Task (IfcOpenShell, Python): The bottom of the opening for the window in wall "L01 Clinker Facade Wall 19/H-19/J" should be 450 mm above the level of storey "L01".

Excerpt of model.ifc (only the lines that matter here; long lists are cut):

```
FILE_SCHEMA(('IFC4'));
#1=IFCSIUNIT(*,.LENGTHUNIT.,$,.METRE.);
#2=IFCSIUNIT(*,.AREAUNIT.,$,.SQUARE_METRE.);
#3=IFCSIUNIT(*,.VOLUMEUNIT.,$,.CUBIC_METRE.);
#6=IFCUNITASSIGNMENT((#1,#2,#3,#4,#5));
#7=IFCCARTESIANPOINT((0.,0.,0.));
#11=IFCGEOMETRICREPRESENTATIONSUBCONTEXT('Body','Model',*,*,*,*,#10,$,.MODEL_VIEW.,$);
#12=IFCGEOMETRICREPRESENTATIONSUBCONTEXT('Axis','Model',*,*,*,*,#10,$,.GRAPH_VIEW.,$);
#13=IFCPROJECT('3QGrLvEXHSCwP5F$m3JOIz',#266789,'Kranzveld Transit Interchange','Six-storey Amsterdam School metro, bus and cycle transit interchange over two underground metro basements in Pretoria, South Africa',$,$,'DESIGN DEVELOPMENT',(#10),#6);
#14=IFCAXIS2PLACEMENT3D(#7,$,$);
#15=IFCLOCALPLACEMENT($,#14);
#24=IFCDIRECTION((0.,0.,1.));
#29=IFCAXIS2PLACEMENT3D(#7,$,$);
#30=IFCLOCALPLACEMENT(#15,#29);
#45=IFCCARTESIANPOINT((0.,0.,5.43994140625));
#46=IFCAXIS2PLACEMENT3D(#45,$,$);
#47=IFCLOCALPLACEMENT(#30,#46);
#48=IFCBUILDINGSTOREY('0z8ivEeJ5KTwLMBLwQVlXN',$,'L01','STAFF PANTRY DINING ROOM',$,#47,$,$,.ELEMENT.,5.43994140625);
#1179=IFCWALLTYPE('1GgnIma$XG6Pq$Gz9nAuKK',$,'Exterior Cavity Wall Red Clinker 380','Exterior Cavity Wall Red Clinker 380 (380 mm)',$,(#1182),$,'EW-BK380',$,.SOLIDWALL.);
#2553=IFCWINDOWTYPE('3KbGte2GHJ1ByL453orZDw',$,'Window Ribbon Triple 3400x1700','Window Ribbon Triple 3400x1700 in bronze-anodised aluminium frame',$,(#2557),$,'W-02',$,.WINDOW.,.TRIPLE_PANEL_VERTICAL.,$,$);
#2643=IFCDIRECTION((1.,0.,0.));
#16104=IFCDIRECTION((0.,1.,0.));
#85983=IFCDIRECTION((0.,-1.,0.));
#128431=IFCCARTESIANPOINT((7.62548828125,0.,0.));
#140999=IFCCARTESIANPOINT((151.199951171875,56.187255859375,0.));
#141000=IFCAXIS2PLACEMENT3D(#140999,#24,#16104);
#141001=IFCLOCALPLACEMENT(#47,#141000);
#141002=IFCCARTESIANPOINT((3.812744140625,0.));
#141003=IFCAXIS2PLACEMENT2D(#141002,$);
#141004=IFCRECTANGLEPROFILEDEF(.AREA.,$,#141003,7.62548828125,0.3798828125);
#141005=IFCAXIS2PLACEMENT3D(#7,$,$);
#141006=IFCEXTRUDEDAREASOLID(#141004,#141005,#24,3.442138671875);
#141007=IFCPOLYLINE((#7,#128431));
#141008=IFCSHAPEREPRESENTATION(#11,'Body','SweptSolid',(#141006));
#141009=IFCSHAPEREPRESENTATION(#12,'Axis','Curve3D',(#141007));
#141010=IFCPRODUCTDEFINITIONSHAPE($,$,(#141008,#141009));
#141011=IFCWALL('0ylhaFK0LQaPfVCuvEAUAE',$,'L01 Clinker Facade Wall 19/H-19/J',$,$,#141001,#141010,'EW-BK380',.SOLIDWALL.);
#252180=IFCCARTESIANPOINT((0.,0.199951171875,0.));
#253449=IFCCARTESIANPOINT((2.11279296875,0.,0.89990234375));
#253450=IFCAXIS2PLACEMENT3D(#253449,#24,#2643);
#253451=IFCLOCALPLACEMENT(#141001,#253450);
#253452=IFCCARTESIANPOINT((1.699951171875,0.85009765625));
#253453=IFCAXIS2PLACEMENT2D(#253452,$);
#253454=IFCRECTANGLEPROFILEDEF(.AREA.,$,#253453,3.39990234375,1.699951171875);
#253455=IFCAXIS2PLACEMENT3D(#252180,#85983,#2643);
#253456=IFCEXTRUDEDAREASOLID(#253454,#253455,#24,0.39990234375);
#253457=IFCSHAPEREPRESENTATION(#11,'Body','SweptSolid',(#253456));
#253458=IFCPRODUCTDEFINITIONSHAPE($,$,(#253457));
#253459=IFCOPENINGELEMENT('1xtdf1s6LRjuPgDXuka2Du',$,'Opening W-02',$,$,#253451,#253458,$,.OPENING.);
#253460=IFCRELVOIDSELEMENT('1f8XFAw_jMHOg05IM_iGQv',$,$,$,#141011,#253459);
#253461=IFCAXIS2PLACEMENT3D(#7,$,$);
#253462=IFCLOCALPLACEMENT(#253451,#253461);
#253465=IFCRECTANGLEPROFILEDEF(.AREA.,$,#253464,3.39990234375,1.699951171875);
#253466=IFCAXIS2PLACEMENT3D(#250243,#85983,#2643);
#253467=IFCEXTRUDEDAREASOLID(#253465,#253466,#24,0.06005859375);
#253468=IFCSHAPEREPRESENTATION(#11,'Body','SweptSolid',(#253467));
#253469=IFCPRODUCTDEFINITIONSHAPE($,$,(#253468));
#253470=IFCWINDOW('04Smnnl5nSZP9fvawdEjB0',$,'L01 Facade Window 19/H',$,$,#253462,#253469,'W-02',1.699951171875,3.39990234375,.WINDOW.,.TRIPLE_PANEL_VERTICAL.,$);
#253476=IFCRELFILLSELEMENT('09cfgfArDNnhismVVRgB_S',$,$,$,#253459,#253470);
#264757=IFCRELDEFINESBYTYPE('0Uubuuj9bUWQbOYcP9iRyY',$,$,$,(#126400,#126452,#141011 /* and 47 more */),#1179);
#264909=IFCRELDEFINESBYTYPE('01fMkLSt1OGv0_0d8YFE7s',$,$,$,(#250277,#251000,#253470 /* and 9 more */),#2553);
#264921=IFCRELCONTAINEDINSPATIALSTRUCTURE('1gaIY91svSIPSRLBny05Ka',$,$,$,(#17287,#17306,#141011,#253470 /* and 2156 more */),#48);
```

```python
import numpy as np
import ifcopenshell
import ifcopenshell.api.geometry
import ifcopenshell.geom
import ifcopenshell.util.element
import ifcopenshell.util.placement
import ifcopenshell.util.shape
import ifcopenshell.util.unit

model = ifcopenshell.open("model.ifc")
unit_scale = ifcopenshell.util.unit.calculate_unit_scale(model)

window = model.by_guid("04Smnnl5nSZP9fvawdEjB0")
opening = window.FillsVoids[0].RelatingOpeningElement
storey = ifcopenshell.util.element.get_container(window, ifc_class="IfcBuildingStorey")
level = ifcopenshell.util.placement.get_local_placement(storey.ObjectPlacement)[2, 3]

# The opening's origin need not be at the sill, so measure its lowest point.
shape = ifcopenshell.geom.create_shape(ifcopenshell.geom.settings(), opening)
bottom = ifcopenshell.util.shape.get_shape_bottom_elevation(shape, shape.geometry) / unit_scale
dz = level + 0.45 - bottom

shift = np.array([0.0, 0.0, dz])
# The window is placed relative to its opening, so it follows when the opening moves.
matrix = ifcopenshell.util.placement.get_local_placement(opening.ObjectPlacement)
matrix[:3, 3] += shift
ifcopenshell.api.geometry.edit_object_placement(
    model, product=opening, matrix=matrix, is_si=False, should_transform_children=True
)

print(f"moved by {dz * unit_scale:+.3f} m")

model.write("model_edited.ifc")
```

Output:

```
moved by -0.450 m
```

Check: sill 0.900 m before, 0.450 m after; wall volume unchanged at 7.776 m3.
